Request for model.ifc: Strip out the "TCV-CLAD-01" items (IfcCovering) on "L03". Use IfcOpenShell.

First a look at what the model holds.

```python
import ifcopenshell
import ifcopenshell.util.element

model = ifcopenshell.open("model.ifc")
print(model.schema)
storey = next(s for s in model.by_type("IfcBuildingStorey") if s.Name == "L03")
coverings = [e for e in ifcopenshell.util.element.get_decomposition(storey) if e.is_a("IfcCovering")]
seen = {}
for e in coverings:
    element_type = ifcopenshell.util.element.get_type(e)
    name = element_type.Name if element_type not in (None, e) else None
    seen[name] = seen.get(name, 0) + 1
for name, count in sorted(seen.items(), key=str):
    print(count, "x", name)
```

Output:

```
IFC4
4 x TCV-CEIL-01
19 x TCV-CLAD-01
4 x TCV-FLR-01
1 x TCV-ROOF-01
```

```python
import ifcopenshell
import ifcopenshell.api.root
import ifcopenshell.util.element

model = ifcopenshell.open("model.ifc")

storey = next(s for s in model.by_type("IfcBuildingStorey") if s.Name == "L03")
coverings = [e for e in ifcopenshell.util.element.get_decomposition(storey) if e.is_a("IfcCovering")]
targets = [e for e in coverings if (t := ifcopenshell.util.element.get_type(e)) not in (None, e) and t.Name == "TCV-CLAD-01"]

for e in targets:
    ifcopenshell.api.root.remove_product(model, product=e)
print(len(targets), "removed")

model.write("model_edited.ifc")
```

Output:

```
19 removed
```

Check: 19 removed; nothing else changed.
